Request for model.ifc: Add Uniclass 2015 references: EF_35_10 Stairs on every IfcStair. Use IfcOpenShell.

First a look at what the model holds.

```python
import ifcopenshell

model = ifcopenshell.open("model.ifc")
print(model.schema)
print("classifications:", [c.Name for c in model.by_type("IfcClassification")])
for ifc_class in ("IfcDoor", "IfcRoof", "IfcStair", "IfcWall", "IfcWindow"):
    print(ifc_class, len(model.by_type(ifc_class)))
```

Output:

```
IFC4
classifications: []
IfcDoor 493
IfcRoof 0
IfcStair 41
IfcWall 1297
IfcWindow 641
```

```python
import ifcopenshell
import ifcopenshell.api.classification

model = ifcopenshell.open("model.ifc")

system = ifcopenshell.api.classification.add_classification(model, classification="Uniclass 2015")

codes = {
    "IfcStair": ("EF_35_10", "Stairs"),
}
for ifc_class, (code, name) in codes.items():
    products = model.by_type(ifc_class)
    ifcopenshell.api.classification.add_reference(
        model, products=products, classification=system, identification=code, name=name
    )
    print(code, len(products))

model.write("model_v2.ifc")
```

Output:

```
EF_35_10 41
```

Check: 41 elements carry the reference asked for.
